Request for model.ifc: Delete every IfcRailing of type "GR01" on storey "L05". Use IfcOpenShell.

First a look at what the model holds.

```python
import ifcopenshell
import ifcopenshell.util.element

model = ifcopenshell.open("model.ifc")
print(model.schema)
storey = next(s for s in model.by_type("IfcBuildingStorey") if s.Name == "L05")
railings = [e for e in ifcopenshell.util.element.get_decomposition(storey) if e.is_a("IfcRailing")]
seen = {}
for e in railings:
    element_type = ifcopenshell.util.element.get_type(e)
    name = element_type.Name if element_type not in (None, e) else None
    seen[name] = seen.get(name, 0) + 1
for name, count in sorted(seen.items(), key=str):
    print(count, "x", name)
```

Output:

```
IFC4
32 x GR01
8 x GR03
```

```python
import ifcopenshell
import ifcopenshell.api.root
import ifcopenshell.util.element

model = ifcopenshell.open("model.ifc")

storey = next(s for s in model.by_type("IfcBuildingStorey") if s.Name == "L05")
railings = [e for e in ifcopenshell.util.element.get_decomposition(storey) if e.is_a("IfcRailing")]
targets = [e for e in railings if (t := ifcopenshell.util.element.get_type(e)) not in (None, e) and t.Name == "GR01"]

for e in targets:
    ifcopenshell.api.root.remove_product(model, product=e)
print(len(targets), "removed")

model.write("model_edited.ifc")
```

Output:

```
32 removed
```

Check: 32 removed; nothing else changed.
